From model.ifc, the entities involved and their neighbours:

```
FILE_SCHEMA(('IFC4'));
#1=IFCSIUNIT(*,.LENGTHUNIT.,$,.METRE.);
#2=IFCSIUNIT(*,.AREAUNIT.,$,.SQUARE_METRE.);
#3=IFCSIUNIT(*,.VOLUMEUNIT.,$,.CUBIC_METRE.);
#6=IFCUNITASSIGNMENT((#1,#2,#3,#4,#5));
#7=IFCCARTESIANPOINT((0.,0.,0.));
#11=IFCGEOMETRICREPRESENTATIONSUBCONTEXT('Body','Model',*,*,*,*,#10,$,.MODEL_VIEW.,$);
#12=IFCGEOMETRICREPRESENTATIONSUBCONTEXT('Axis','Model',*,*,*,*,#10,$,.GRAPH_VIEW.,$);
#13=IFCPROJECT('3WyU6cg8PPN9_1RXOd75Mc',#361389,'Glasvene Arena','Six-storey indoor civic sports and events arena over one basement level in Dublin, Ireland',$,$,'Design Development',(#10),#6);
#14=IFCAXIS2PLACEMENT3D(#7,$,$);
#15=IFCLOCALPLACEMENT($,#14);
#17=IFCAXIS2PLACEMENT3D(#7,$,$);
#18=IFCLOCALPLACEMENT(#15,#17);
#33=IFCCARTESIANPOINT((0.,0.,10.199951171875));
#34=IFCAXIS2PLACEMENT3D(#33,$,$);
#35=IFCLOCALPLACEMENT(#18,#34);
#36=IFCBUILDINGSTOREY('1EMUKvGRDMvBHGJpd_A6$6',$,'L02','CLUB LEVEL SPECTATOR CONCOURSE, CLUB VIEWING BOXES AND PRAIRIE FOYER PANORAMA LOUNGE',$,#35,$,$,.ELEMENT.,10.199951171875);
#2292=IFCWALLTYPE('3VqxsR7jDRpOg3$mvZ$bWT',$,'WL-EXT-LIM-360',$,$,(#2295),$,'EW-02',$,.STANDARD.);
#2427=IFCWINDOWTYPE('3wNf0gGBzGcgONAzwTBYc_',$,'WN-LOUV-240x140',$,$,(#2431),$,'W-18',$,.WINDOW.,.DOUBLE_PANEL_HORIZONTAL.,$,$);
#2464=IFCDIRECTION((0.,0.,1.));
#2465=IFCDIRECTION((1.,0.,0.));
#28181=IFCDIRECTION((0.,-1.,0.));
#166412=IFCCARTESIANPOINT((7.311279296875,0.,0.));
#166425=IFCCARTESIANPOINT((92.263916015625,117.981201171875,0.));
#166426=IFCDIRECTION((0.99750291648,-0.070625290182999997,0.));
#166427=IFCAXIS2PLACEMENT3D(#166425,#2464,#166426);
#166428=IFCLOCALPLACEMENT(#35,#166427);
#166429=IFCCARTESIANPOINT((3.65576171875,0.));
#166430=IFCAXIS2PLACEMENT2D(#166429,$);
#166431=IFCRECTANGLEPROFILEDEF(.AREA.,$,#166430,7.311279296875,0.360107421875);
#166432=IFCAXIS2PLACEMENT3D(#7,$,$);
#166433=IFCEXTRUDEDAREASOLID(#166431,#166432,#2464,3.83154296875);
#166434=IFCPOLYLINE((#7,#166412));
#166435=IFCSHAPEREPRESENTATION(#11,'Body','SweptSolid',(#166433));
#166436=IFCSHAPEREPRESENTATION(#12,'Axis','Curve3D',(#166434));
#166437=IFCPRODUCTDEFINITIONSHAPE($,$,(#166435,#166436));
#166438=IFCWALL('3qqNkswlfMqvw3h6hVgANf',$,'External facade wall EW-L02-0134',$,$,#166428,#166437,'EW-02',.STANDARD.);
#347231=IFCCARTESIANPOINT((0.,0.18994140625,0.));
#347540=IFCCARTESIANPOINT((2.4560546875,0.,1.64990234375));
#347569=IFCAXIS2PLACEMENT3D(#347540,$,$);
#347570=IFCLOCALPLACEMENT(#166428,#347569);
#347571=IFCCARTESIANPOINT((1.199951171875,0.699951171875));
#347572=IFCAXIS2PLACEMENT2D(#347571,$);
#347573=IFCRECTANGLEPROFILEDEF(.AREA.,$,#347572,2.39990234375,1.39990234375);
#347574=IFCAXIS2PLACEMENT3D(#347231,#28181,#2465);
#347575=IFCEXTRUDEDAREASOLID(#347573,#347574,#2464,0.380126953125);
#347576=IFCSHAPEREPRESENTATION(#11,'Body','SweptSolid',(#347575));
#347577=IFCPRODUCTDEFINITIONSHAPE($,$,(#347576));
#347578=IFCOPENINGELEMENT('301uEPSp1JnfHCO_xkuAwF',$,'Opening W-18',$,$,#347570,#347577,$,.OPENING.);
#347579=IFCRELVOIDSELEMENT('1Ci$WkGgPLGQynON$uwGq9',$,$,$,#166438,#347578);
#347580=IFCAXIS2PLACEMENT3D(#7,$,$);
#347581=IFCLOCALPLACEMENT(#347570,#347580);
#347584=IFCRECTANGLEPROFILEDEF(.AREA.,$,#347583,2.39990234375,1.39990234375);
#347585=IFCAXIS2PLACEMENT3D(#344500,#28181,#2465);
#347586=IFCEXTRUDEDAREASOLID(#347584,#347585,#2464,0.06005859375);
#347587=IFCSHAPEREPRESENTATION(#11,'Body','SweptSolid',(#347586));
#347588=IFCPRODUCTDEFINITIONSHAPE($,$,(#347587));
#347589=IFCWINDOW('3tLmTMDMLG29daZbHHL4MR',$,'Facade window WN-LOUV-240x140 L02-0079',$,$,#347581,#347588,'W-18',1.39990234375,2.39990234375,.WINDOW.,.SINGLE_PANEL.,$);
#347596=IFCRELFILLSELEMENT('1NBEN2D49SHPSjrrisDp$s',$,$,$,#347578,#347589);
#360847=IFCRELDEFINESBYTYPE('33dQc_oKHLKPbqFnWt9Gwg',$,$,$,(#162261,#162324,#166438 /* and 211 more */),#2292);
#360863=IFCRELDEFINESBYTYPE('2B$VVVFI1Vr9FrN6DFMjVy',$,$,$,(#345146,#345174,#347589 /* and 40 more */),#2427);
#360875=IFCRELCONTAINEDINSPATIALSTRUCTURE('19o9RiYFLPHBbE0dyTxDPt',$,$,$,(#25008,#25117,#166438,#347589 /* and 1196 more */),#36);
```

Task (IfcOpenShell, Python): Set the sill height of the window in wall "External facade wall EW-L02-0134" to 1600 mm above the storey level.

```python
import numpy as np
import ifcopenshell
import ifcopenshell.api.geometry
import ifcopenshell.geom
import ifcopenshell.util.element
import ifcopenshell.util.placement
import ifcopenshell.util.shape
import ifcopenshell.util.unit

model = ifcopenshell.open("model.ifc")
unit_scale = ifcopenshell.util.unit.calculate_unit_scale(model)

window = model.by_guid("3tLmTMDMLG29daZbHHL4MR")
opening = window.FillsVoids[0].RelatingOpeningElement
storey = ifcopenshell.util.element.get_container(window, ifc_class="IfcBuildingStorey")
level = ifcopenshell.util.placement.get_local_placement(storey.ObjectPlacement)[2, 3]

# The opening's origin need not be at the sill, so measure its lowest point.
shape = ifcopenshell.geom.create_shape(ifcopenshell.geom.settings(), opening)
bottom = ifcopenshell.util.shape.get_shape_bottom_elevation(shape, shape.geometry) / unit_scale
dz = level + 1.6 / unit_scale - bottom

shift = np.array([0.0, 0.0, dz])
# The window is placed relative to its opening, so it follows when the opening moves.
matrix = ifcopenshell.util.placement.get_local_placement(opening.ObjectPlacement)
matrix[:3, 3] += shift
ifcopenshell.api.geometry.edit_object_placement(
    model, product=opening, matrix=matrix, is_si=False, should_transform_children=True
)

print(f"moved by {dz * unit_scale:+.3f} m")

model.write("model-out.ifc")
```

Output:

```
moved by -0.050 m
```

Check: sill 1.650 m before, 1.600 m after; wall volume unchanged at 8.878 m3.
